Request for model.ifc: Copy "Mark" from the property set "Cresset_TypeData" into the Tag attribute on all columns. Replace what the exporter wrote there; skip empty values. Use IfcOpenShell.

First a look at what the model holds.

```python
import ifcopenshell
import ifcopenshell.util.element

model = ifcopenshell.open("model.ifc")
print(model.schema)
columns = model.by_type("IfcColumn")
print(len(columns), "columns")
for e in columns[:8]:
    source = ifcopenshell.util.element.get_pset(e, "Cresset_TypeData", "Mark")
    target = e.Tag
    print(e.id(), repr(source), repr(target), sep=" | ")
```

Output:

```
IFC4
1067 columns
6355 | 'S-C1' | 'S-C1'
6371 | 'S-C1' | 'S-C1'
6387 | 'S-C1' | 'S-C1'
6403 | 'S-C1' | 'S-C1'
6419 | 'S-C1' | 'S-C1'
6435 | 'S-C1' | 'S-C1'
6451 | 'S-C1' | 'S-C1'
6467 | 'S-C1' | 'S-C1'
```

```python
import ifcopenshell
import ifcopenshell.util.element

model = ifcopenshell.open("model.ifc")

count = 0
for e in model.by_type("IfcColumn"):
    value = ifcopenshell.util.element.get_pset(e, "Cresset_TypeData", "Mark")
    current = e.Tag
    if not value or not value.strip() or current == value:
        continue
    e.Tag = value
    count += 1

print(count, "columns updated")

model.write("model_rev.ifc")
```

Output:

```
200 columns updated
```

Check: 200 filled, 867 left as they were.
